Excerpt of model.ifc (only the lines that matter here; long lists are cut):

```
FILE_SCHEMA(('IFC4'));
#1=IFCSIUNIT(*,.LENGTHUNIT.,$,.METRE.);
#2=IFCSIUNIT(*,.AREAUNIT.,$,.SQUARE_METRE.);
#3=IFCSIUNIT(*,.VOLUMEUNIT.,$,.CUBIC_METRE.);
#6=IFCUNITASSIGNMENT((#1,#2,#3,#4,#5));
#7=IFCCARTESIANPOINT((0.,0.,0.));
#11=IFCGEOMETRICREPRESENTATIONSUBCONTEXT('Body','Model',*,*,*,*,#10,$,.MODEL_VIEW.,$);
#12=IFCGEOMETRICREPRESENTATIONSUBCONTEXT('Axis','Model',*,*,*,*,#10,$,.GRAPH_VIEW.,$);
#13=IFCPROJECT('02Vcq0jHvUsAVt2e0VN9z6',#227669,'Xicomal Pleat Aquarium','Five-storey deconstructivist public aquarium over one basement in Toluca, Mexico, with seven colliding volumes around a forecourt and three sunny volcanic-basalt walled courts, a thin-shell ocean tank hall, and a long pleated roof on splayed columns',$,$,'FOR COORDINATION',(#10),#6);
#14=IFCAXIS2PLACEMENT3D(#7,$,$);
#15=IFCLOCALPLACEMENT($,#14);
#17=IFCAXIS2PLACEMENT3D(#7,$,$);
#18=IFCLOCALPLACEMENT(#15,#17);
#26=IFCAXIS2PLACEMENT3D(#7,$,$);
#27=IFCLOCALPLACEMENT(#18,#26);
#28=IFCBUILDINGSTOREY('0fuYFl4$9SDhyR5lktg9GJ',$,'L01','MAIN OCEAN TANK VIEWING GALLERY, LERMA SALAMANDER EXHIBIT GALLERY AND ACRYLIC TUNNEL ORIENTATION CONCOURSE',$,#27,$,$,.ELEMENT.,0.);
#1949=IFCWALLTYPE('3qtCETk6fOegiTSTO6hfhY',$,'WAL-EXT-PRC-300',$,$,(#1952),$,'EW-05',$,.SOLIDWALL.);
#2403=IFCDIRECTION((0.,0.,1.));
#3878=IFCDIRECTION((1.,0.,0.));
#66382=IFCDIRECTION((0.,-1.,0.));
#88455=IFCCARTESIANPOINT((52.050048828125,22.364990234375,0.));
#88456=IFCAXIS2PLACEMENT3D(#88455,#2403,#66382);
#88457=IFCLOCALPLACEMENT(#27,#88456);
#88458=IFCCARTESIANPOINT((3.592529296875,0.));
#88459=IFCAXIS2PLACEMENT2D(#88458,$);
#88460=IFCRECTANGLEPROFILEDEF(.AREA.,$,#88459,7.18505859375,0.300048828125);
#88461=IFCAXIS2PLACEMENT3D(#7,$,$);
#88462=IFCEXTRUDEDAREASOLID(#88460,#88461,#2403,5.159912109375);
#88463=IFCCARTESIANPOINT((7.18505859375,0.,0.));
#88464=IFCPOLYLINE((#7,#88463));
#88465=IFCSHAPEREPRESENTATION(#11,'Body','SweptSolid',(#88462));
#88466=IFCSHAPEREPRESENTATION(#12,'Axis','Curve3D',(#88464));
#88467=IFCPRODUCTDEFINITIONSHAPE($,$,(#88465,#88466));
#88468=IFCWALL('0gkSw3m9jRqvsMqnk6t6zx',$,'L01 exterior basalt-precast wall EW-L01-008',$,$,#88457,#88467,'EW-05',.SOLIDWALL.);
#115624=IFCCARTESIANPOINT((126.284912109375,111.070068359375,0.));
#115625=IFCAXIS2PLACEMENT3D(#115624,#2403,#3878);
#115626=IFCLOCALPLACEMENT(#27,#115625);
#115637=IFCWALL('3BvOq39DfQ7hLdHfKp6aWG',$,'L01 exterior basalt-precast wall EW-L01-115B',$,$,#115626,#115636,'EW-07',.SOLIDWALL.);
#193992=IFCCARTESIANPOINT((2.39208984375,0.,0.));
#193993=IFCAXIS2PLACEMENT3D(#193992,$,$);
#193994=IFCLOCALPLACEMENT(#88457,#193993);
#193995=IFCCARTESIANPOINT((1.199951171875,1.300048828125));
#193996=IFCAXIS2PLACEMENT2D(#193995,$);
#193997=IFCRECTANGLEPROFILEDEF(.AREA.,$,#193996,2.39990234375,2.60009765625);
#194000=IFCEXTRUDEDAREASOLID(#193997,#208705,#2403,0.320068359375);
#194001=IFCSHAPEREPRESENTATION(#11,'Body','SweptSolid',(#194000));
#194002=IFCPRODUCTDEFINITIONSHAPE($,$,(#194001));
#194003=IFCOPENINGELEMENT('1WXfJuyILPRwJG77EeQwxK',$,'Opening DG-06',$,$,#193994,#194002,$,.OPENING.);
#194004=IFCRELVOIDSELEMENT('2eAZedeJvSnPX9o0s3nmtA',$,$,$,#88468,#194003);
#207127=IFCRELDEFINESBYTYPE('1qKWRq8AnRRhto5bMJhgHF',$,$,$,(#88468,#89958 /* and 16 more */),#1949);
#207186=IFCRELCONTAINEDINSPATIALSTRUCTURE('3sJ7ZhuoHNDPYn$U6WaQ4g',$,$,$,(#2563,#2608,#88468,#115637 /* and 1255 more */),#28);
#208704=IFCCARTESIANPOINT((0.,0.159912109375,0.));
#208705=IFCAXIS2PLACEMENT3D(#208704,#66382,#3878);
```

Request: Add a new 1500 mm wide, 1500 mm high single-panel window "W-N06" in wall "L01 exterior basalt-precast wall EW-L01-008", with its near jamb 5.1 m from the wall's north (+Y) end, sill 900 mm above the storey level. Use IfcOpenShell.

```python
import numpy as np
import ifcopenshell
import ifcopenshell.api.feature
import ifcopenshell.api.geometry
import ifcopenshell.api.root
import ifcopenshell.api.spatial
import ifcopenshell.geom
import ifcopenshell.util.element
import ifcopenshell.util.placement
import ifcopenshell.util.representation
import ifcopenshell.util.shape
import ifcopenshell.util.unit

model = ifcopenshell.open("model.ifc")
unit_scale = ifcopenshell.util.unit.calculate_unit_scale(model)
settings = ifcopenshell.geom.settings()


def volume(element):
    """Net volume in cubic metres, openings subtracted."""
    shape = ifcopenshell.geom.create_shape(settings, element)
    return ifcopenshell.util.shape.get_volume(shape.geometry)


wall = model.by_guid("0gkSw3m9jRqvsMqnk6t6zx")
storey = ifcopenshell.util.element.get_container(wall, ifc_class="IfcBuildingStorey")
context = ifcopenshell.util.representation.get_context(model, "Model", "Body", "MODEL_VIEW")
before = volume(wall)

width, height, from_end, sill = 1.5, 1.5, 5.1, 0.9  # metres

# The wall runs along its own X axis, and the end named is its -X end.
wall_shape = ifcopenshell.geom.create_shape(settings, wall)
x, y, z = ifcopenshell.util.shape.get_vertices(wall_shape.geometry).T
start = x.min() + from_end
face, thickness = float(y.min()), float(y.max() - y.min())
wall_matrix = ifcopenshell.util.placement.get_local_placement(wall.ObjectPlacement)
level = ifcopenshell.util.placement.get_local_placement(storey.ObjectPlacement)[2, 3]


def in_wall(x, y):
    """Placement at x, y metres in the wall's axes, at sill height."""
    matrix = wall_matrix.copy()
    matrix[:, 3] = wall_matrix @ np.array([x / unit_scale, y / unit_scale, 0.0, 1.0])
    matrix[2, 3] = level + sill / unit_scale
    return matrix


# Opening: a box that overshoots both wall faces by 50 mm.
opening = ifcopenshell.api.root.create_entity(model, ifc_class="IfcOpeningElement", predefined_type="OPENING")
box = ifcopenshell.api.geometry.add_wall_representation(
    model, context=context, length=width, height=height, thickness=thickness + 0.1
)
ifcopenshell.api.geometry.assign_representation(model, product=opening, representation=box)
ifcopenshell.api.geometry.edit_object_placement(model, product=opening, matrix=in_wall(start, face - 0.05), is_si=False)
ifcopenshell.api.feature.add_feature(model, feature=opening, element=wall)

window = ifcopenshell.api.root.create_entity(model, ifc_class="IfcWindow", name="W-N06", predefined_type="WINDOW")
window.OverallWidth, window.OverallHeight = width / unit_scale, height / unit_scale
window.PartitioningType = "SINGLE_PANEL"
body = ifcopenshell.api.geometry.add_window_representation(
    model,
    context=context,
    overall_width=window.OverallWidth,
    overall_height=window.OverallHeight,
    partition_type="SINGLE_PANEL",
)
ifcopenshell.api.geometry.assign_representation(model, product=window, representation=body)
ifcopenshell.api.spatial.assign_container(model, products=[window], relating_structure=storey)
ifcopenshell.api.feature.add_filling(model, opening=opening, element=window)

# Centre the window in the wall's thickness.
ifcopenshell.api.geometry.edit_object_placement(model, product=window, matrix=in_wall(start, face), is_si=False)
window_shape = ifcopenshell.geom.create_shape(settings, window)
depth = ifcopenshell.util.shape.get_vertices(window_shape.geometry)[:, 1]
offset = face + thickness / 2 - (depth.min() + depth.max()) / 2
ifcopenshell.api.geometry.edit_object_placement(model, product=window, matrix=in_wall(start, offset), is_si=False)

after = volume(wall)

print(f"wall volume {before:.3f} -> {after:.3f} m3")

model.write("model-out.ifc")
```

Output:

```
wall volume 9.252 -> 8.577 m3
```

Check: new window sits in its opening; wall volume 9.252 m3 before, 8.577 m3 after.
